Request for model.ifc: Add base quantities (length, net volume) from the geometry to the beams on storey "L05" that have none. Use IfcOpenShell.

First a look at what the model holds.

```python
import ifcopenshell
import ifcopenshell.util.element
import ifcopenshell.util.unit

model = ifcopenshell.open("model.ifc")
print(model.schema)
for unit_type in ("LENGTHUNIT", "AREAUNIT", "VOLUMEUNIT"):
    print(unit_type, ifcopenshell.util.unit.calculate_unit_scale(model, unit_type))
storey = next(s for s in model.by_type("IfcBuildingStorey") if s.Name == "L05")
beams = [e for e in ifcopenshell.util.element.get_decomposition(storey) if e.is_a("IfcBeam")]
for e in sorted(beams, key=lambda e: e.id()):
    print(e.id(), e.is_a(), e.Name, list(ifcopenshell.util.element.get_psets(e, qtos_only=True)), sep=" | ")
```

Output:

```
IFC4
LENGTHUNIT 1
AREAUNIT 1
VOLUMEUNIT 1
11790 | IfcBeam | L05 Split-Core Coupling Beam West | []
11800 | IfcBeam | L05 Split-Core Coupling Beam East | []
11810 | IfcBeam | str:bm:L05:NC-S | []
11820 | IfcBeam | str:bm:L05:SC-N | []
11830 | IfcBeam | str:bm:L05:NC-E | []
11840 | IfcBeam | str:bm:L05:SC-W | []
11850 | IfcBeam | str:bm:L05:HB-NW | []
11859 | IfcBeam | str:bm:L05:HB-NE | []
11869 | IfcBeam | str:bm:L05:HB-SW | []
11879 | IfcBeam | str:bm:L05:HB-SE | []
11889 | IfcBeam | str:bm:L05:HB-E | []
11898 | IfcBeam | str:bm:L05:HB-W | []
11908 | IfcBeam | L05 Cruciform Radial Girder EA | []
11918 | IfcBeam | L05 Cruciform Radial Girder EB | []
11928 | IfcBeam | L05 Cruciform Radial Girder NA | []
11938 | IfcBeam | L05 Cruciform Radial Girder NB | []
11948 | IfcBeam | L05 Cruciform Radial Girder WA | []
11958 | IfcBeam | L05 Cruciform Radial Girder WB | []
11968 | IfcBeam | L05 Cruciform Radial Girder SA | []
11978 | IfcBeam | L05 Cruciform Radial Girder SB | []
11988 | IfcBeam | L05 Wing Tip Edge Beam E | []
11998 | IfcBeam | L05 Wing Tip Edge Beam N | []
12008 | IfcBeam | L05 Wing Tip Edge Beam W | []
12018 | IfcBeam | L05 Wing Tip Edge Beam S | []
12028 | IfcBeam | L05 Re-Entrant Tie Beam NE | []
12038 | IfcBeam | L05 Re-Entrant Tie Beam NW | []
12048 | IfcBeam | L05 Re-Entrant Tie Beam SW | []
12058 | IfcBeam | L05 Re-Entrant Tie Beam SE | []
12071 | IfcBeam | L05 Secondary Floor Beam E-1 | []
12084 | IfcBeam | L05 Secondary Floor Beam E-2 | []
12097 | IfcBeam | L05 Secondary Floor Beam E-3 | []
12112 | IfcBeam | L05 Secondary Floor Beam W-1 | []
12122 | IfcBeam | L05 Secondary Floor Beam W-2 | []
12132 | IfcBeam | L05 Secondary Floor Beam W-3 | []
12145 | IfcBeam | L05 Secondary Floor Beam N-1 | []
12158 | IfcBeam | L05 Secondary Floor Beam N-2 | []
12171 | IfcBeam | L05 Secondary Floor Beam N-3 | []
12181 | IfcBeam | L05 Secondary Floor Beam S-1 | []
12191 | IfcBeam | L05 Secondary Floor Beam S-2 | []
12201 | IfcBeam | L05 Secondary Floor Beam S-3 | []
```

```python
import ifcopenshell
import ifcopenshell.api.pset
import ifcopenshell.geom
import ifcopenshell.util.element
import ifcopenshell.util.shape
import ifcopenshell.util.unit

model = ifcopenshell.open("model.ifc")
unit_scale = ifcopenshell.util.unit.calculate_unit_scale(model)
volume_scale = ifcopenshell.util.unit.calculate_unit_scale(model, "VOLUMEUNIT")
settings = ifcopenshell.geom.settings()

storey = next(s for s in model.by_type("IfcBuildingStorey") if s.Name == "L05")
beams = [e for e in ifcopenshell.util.element.get_decomposition(storey) if e.is_a("IfcBeam")]

for e in sorted(beams, key=lambda e: e.id()):
    if ifcopenshell.util.element.get_psets(e, qtos_only=True, should_inherit=False):
        continue
    # Geometry comes back in metres, in the element's own axes.
    shape = ifcopenshell.geom.create_shape(settings, e)
    values = {
        "Length": ifcopenshell.util.shape.get_max_xyz(shape.geometry) / unit_scale,
        "NetVolume": ifcopenshell.util.shape.get_volume(shape.geometry) / volume_scale,
    }
    qto = ifcopenshell.api.pset.add_qto(model, product=e, name="Qto_BeamBaseQuantities")
    ifcopenshell.api.pset.edit_qto(model, qto=qto, properties=values)
    print(e.id(), {k: round(v, 3) for k, v in values.items()})

model.write("model_updated.ifc")
```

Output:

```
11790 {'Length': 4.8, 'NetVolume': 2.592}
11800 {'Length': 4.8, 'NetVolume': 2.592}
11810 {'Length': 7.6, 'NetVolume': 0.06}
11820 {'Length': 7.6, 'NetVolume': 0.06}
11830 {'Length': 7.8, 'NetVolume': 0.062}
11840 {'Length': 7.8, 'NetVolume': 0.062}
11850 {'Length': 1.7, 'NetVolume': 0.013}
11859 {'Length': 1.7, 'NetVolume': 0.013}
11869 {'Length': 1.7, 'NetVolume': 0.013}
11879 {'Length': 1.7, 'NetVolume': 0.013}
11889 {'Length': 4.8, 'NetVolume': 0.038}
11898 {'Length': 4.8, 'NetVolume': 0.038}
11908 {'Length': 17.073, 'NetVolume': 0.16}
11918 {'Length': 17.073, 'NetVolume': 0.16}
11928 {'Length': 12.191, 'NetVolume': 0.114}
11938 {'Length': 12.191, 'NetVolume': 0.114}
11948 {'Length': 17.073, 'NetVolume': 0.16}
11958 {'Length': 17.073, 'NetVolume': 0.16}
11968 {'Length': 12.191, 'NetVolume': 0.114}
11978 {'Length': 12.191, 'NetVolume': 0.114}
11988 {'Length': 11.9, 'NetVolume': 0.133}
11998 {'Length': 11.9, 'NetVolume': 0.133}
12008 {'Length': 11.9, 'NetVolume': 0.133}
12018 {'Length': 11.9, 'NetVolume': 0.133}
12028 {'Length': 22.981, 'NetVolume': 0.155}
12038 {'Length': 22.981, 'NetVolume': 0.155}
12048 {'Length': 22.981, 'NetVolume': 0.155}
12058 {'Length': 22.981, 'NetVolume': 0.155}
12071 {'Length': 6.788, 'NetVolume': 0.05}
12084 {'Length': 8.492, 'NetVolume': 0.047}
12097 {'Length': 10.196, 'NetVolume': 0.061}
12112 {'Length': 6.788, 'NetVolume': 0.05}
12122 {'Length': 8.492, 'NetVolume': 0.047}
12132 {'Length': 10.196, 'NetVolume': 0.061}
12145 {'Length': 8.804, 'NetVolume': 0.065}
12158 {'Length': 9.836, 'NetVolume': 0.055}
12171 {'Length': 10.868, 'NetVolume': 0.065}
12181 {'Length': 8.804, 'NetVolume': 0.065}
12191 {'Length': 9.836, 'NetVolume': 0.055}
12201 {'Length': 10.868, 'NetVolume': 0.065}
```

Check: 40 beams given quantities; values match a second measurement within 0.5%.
